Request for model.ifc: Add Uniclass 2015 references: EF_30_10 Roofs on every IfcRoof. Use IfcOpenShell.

First a look at what the model holds.

```python
import ifcopenshell

model = ifcopenshell.open("model.ifc")
print(model.schema)
print("classifications:", [c.Name for c in model.by_type("IfcClassification")])
for ifc_class in ("IfcDoor", "IfcRoof", "IfcStair", "IfcWall", "IfcWindow"):
    print(ifc_class, len(model.by_type(ifc_class)))
```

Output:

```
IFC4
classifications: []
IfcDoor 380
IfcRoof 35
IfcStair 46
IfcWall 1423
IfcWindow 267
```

```python
import ifcopenshell
import ifcopenshell.api.classification

model = ifcopenshell.open("model.ifc")

system = ifcopenshell.api.classification.add_classification(model, classification="Uniclass 2015")

codes = {
    "IfcRoof": ("EF_30_10", "Roofs"),
}
for ifc_class, (code, name) in codes.items():
    products = model.by_type(ifc_class)
    ifcopenshell.api.classification.add_reference(
        model, products=products, classification=system, identification=code, name=name
    )
    print(code, len(products))

model.write("model_rev.ifc")
```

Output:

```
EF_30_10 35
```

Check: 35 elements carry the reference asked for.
